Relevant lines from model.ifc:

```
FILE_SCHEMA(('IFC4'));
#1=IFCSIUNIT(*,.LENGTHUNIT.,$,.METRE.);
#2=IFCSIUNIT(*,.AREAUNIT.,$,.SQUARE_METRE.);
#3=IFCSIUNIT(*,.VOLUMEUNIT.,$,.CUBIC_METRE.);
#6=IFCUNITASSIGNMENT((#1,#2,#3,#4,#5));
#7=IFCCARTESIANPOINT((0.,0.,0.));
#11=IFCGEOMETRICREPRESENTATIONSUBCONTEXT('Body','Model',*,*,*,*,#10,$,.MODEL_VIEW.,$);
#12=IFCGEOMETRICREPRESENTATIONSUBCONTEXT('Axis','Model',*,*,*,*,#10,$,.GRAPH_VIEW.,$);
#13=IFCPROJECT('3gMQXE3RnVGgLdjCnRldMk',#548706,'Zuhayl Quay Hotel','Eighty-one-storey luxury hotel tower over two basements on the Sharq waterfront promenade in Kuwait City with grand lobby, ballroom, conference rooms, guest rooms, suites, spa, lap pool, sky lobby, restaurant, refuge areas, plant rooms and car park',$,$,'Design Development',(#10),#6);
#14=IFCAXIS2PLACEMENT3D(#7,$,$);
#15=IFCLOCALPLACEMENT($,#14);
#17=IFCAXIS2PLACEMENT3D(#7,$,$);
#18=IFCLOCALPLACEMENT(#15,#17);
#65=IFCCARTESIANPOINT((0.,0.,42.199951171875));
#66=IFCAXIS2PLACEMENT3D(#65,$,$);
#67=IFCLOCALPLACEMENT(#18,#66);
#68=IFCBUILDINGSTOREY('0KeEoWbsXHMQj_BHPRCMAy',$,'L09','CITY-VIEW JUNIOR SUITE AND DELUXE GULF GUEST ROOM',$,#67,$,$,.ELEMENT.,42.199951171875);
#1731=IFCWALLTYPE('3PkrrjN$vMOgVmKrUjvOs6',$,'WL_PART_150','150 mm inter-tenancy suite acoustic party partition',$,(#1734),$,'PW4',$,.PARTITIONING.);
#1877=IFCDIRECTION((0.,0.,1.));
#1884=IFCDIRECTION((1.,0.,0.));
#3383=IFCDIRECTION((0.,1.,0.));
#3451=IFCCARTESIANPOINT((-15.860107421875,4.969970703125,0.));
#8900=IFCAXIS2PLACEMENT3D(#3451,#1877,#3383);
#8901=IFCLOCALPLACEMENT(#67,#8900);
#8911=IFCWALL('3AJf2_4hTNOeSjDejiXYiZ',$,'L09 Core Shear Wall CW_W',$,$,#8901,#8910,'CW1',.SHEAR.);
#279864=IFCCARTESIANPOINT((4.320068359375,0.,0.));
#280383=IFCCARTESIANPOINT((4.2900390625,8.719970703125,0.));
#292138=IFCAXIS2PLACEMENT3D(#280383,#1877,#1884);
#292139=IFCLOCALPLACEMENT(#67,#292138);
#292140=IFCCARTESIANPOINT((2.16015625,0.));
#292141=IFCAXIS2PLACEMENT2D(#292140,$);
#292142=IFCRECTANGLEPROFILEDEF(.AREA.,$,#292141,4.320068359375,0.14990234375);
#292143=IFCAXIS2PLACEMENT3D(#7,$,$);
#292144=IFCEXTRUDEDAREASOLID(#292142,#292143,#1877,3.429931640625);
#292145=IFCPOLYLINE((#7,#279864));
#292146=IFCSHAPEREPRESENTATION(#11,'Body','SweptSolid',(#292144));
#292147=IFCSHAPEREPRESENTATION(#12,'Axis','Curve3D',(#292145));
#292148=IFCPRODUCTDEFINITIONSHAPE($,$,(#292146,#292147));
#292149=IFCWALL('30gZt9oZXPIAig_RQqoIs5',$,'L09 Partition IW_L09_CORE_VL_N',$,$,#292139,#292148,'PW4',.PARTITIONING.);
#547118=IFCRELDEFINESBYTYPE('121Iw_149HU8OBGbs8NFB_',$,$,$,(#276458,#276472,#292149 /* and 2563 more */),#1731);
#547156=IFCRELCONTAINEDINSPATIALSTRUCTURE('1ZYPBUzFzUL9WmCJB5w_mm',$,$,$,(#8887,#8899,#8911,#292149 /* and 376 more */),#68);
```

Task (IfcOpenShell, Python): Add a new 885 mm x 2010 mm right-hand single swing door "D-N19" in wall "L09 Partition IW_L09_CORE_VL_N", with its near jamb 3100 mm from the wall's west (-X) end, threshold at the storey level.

```python
import numpy as np
import ifcopenshell
import ifcopenshell.api.feature
import ifcopenshell.api.geometry
import ifcopenshell.api.root
import ifcopenshell.api.spatial
import ifcopenshell.geom
import ifcopenshell.util.element
import ifcopenshell.util.placement
import ifcopenshell.util.representation
import ifcopenshell.util.shape
import ifcopenshell.util.unit

model = ifcopenshell.open("model.ifc")
unit_scale = ifcopenshell.util.unit.calculate_unit_scale(model)
settings = ifcopenshell.geom.settings()


def volume(element):
    """Net volume in cubic metres, openings subtracted."""
    shape = ifcopenshell.geom.create_shape(settings, element)
    return ifcopenshell.util.shape.get_volume(shape.geometry)


wall = model.by_guid("30gZt9oZXPIAig_RQqoIs5")
storey = ifcopenshell.util.element.get_container(wall, ifc_class="IfcBuildingStorey")
context = ifcopenshell.util.representation.get_context(model, "Model", "Body", "MODEL_VIEW")
before = volume(wall)

width, height, from_end, sill = 0.885, 2.01, 3.1, 0.0  # metres

# The wall runs along its own X axis, and the end named is its -X end.
wall_shape = ifcopenshell.geom.create_shape(settings, wall)
x, y, z = ifcopenshell.util.shape.get_vertices(wall_shape.geometry).T
start = x.min() + from_end
face, thickness = float(y.min()), float(y.max() - y.min())
wall_matrix = ifcopenshell.util.placement.get_local_placement(wall.ObjectPlacement)
level = ifcopenshell.util.placement.get_local_placement(storey.ObjectPlacement)[2, 3]


def in_wall(x, y):
    """Placement at x, y metres in the wall's axes, at sill height."""
    matrix = wall_matrix.copy()
    matrix[:, 3] = wall_matrix @ np.array([x / unit_scale, y / unit_scale, 0.0, 1.0])
    matrix[2, 3] = level + sill / unit_scale
    return matrix


# Opening: a box that overshoots both wall faces by 50 mm.
opening = ifcopenshell.api.root.create_entity(model, ifc_class="IfcOpeningElement", predefined_type="OPENING")
box = ifcopenshell.api.geometry.add_wall_representation(
    model, context=context, length=width, height=height, thickness=thickness + 0.1
)
ifcopenshell.api.geometry.assign_representation(model, product=opening, representation=box)
ifcopenshell.api.geometry.edit_object_placement(model, product=opening, matrix=in_wall(start, face - 0.05), is_si=False)
ifcopenshell.api.feature.add_feature(model, feature=opening, element=wall)

door = ifcopenshell.api.root.create_entity(model, ifc_class="IfcDoor", name="D-N19", predefined_type="DOOR")
door.OverallWidth, door.OverallHeight = width / unit_scale, height / unit_scale
door.OperationType = "SINGLE_SWING_RIGHT"
body = ifcopenshell.api.geometry.add_door_representation(
    model,
    context=context,
    overall_width=door.OverallWidth,
    overall_height=door.OverallHeight,
    operation_type="SINGLE_SWING_RIGHT",
    lining_properties={"LiningDepth": thickness / unit_scale, "ThresholdDepth": thickness / unit_scale},
)
ifcopenshell.api.geometry.assign_representation(model, product=door, representation=body)
ifcopenshell.api.spatial.assign_container(model, products=[door], relating_structure=storey)
ifcopenshell.api.feature.add_filling(model, opening=opening, element=door)

# The lining spans the wall, so the door starts at the wall face.
ifcopenshell.api.geometry.edit_object_placement(model, product=door, matrix=in_wall(start, face), is_si=False)

after = volume(wall)

print(f"wall volume {before:.3f} -> {after:.3f} m3")

model.write("model_updated.ifc")
```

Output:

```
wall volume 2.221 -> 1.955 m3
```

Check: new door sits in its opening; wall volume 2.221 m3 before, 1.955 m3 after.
